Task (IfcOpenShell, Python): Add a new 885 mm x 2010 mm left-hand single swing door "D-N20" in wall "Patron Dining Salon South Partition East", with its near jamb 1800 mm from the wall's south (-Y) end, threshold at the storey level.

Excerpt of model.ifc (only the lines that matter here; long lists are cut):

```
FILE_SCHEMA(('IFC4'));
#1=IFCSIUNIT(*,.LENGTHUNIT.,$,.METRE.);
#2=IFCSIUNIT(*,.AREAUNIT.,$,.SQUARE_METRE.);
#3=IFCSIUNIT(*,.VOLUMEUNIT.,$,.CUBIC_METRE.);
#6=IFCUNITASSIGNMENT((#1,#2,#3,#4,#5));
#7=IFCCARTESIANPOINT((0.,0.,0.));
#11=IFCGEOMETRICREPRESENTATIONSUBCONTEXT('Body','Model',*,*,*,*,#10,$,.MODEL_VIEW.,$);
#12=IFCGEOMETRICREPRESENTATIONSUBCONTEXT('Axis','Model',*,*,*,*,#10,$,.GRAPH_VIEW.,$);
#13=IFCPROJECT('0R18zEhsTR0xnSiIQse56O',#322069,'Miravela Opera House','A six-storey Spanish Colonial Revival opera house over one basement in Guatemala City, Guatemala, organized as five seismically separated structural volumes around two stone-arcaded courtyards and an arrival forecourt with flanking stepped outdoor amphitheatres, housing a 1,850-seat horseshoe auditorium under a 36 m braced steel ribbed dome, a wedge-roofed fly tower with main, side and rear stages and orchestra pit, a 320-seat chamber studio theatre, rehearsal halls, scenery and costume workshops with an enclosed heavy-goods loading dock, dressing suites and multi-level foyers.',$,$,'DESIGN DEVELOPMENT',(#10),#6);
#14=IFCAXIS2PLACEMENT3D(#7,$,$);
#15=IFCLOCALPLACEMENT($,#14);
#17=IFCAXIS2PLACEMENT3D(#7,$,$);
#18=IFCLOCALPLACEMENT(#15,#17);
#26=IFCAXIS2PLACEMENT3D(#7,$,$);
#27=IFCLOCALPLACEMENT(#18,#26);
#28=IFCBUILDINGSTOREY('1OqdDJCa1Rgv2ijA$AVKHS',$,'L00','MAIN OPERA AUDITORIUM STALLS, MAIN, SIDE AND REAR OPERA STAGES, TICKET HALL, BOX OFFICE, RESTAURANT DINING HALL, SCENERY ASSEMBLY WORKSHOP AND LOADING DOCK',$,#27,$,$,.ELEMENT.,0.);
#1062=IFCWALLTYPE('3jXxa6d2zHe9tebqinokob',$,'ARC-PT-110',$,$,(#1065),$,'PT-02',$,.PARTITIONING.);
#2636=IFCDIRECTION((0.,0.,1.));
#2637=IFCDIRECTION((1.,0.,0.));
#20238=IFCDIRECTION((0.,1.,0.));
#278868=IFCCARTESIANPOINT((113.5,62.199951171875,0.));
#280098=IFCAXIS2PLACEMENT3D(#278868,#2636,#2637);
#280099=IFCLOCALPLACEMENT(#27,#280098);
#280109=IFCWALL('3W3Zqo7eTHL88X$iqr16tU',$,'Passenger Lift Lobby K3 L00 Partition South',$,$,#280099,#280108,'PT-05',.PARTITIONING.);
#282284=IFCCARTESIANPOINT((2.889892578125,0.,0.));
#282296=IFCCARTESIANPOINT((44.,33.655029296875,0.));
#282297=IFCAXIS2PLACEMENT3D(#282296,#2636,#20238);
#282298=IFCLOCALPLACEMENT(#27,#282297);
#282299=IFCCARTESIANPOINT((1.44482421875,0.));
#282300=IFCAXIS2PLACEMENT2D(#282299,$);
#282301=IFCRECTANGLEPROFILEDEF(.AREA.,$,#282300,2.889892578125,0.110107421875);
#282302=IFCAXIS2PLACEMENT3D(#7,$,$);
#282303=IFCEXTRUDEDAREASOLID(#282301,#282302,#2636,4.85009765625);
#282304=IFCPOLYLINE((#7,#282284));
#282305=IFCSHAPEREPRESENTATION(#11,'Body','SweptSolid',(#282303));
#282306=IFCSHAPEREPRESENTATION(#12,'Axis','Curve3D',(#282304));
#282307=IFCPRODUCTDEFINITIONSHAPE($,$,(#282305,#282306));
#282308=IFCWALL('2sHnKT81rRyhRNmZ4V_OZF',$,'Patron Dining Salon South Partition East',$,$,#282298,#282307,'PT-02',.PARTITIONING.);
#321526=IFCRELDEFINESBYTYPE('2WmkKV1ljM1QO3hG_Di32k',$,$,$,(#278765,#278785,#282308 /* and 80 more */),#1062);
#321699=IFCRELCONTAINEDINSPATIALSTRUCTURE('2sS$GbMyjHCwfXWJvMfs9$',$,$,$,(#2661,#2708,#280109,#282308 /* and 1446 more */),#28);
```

```python
import numpy as np
import ifcopenshell
import ifcopenshell.api.feature
import ifcopenshell.api.geometry
import ifcopenshell.api.root
import ifcopenshell.api.spatial
import ifcopenshell.geom
import ifcopenshell.util.element
import ifcopenshell.util.placement
import ifcopenshell.util.representation
import ifcopenshell.util.shape
import ifcopenshell.util.unit

model = ifcopenshell.open("model.ifc")
unit_scale = ifcopenshell.util.unit.calculate_unit_scale(model)
settings = ifcopenshell.geom.settings()


def volume(element):
    """Net volume in cubic metres, openings subtracted."""
    shape = ifcopenshell.geom.create_shape(settings, element)
    return ifcopenshell.util.shape.get_volume(shape.geometry)


wall = model.by_guid("2sHnKT81rRyhRNmZ4V_OZF")
storey = ifcopenshell.util.element.get_container(wall, ifc_class="IfcBuildingStorey")
context = ifcopenshell.util.representation.get_context(model, "Model", "Body", "MODEL_VIEW")
before = volume(wall)

width, height, from_end, sill = 0.885, 2.01, 1.8, 0.0  # metres

# The wall runs along its own X axis, and the end named is its -X end.
wall_shape = ifcopenshell.geom.create_shape(settings, wall)
x, y, z = ifcopenshell.util.shape.get_vertices(wall_shape.geometry).T
start = x.min() + from_end
face, thickness = float(y.min()), float(y.max() - y.min())
wall_matrix = ifcopenshell.util.placement.get_local_placement(wall.ObjectPlacement)
level = ifcopenshell.util.placement.get_local_placement(storey.ObjectPlacement)[2, 3]


def in_wall(x, y):
    """Placement at x, y metres in the wall's axes, at sill height."""
    matrix = wall_matrix.copy()
    matrix[:, 3] = wall_matrix @ np.array([x / unit_scale, y / unit_scale, 0.0, 1.0])
    matrix[2, 3] = level + sill / unit_scale
    return matrix


# Opening: a box that overshoots both wall faces by 50 mm.
opening = ifcopenshell.api.root.create_entity(model, ifc_class="IfcOpeningElement", predefined_type="OPENING")
box = ifcopenshell.api.geometry.add_wall_representation(
    model, context=context, length=width, height=height, thickness=thickness + 0.1
)
ifcopenshell.api.geometry.assign_representation(model, product=opening, representation=box)
ifcopenshell.api.geometry.edit_object_placement(model, product=opening, matrix=in_wall(start, face - 0.05), is_si=False)
ifcopenshell.api.feature.add_feature(model, feature=opening, element=wall)

door = ifcopenshell.api.root.create_entity(model, ifc_class="IfcDoor", name="D-N20", predefined_type="DOOR")
door.OverallWidth, door.OverallHeight = width / unit_scale, height / unit_scale
door.OperationType = "SINGLE_SWING_LEFT"
body = ifcopenshell.api.geometry.add_door_representation(
    model,
    context=context,
    overall_width=door.OverallWidth,
    overall_height=door.OverallHeight,
    operation_type="SINGLE_SWING_LEFT",
    lining_properties={"LiningDepth": thickness / unit_scale, "ThresholdDepth": thickness / unit_scale},
)
ifcopenshell.api.geometry.assign_representation(model, product=door, representation=body)
ifcopenshell.api.spatial.assign_container(model, products=[door], relating_structure=storey)
ifcopenshell.api.feature.add_filling(model, opening=opening, element=door)

# The lining spans the wall, so the door starts at the wall face.
ifcopenshell.api.geometry.edit_object_placement(model, product=door, matrix=in_wall(start, face), is_si=False)

after = volume(wall)

print(f"wall volume {before:.3f} -> {after:.3f} m3")

model.write("model_v2.ifc")
```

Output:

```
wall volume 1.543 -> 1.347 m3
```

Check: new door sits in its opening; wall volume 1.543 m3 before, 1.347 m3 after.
